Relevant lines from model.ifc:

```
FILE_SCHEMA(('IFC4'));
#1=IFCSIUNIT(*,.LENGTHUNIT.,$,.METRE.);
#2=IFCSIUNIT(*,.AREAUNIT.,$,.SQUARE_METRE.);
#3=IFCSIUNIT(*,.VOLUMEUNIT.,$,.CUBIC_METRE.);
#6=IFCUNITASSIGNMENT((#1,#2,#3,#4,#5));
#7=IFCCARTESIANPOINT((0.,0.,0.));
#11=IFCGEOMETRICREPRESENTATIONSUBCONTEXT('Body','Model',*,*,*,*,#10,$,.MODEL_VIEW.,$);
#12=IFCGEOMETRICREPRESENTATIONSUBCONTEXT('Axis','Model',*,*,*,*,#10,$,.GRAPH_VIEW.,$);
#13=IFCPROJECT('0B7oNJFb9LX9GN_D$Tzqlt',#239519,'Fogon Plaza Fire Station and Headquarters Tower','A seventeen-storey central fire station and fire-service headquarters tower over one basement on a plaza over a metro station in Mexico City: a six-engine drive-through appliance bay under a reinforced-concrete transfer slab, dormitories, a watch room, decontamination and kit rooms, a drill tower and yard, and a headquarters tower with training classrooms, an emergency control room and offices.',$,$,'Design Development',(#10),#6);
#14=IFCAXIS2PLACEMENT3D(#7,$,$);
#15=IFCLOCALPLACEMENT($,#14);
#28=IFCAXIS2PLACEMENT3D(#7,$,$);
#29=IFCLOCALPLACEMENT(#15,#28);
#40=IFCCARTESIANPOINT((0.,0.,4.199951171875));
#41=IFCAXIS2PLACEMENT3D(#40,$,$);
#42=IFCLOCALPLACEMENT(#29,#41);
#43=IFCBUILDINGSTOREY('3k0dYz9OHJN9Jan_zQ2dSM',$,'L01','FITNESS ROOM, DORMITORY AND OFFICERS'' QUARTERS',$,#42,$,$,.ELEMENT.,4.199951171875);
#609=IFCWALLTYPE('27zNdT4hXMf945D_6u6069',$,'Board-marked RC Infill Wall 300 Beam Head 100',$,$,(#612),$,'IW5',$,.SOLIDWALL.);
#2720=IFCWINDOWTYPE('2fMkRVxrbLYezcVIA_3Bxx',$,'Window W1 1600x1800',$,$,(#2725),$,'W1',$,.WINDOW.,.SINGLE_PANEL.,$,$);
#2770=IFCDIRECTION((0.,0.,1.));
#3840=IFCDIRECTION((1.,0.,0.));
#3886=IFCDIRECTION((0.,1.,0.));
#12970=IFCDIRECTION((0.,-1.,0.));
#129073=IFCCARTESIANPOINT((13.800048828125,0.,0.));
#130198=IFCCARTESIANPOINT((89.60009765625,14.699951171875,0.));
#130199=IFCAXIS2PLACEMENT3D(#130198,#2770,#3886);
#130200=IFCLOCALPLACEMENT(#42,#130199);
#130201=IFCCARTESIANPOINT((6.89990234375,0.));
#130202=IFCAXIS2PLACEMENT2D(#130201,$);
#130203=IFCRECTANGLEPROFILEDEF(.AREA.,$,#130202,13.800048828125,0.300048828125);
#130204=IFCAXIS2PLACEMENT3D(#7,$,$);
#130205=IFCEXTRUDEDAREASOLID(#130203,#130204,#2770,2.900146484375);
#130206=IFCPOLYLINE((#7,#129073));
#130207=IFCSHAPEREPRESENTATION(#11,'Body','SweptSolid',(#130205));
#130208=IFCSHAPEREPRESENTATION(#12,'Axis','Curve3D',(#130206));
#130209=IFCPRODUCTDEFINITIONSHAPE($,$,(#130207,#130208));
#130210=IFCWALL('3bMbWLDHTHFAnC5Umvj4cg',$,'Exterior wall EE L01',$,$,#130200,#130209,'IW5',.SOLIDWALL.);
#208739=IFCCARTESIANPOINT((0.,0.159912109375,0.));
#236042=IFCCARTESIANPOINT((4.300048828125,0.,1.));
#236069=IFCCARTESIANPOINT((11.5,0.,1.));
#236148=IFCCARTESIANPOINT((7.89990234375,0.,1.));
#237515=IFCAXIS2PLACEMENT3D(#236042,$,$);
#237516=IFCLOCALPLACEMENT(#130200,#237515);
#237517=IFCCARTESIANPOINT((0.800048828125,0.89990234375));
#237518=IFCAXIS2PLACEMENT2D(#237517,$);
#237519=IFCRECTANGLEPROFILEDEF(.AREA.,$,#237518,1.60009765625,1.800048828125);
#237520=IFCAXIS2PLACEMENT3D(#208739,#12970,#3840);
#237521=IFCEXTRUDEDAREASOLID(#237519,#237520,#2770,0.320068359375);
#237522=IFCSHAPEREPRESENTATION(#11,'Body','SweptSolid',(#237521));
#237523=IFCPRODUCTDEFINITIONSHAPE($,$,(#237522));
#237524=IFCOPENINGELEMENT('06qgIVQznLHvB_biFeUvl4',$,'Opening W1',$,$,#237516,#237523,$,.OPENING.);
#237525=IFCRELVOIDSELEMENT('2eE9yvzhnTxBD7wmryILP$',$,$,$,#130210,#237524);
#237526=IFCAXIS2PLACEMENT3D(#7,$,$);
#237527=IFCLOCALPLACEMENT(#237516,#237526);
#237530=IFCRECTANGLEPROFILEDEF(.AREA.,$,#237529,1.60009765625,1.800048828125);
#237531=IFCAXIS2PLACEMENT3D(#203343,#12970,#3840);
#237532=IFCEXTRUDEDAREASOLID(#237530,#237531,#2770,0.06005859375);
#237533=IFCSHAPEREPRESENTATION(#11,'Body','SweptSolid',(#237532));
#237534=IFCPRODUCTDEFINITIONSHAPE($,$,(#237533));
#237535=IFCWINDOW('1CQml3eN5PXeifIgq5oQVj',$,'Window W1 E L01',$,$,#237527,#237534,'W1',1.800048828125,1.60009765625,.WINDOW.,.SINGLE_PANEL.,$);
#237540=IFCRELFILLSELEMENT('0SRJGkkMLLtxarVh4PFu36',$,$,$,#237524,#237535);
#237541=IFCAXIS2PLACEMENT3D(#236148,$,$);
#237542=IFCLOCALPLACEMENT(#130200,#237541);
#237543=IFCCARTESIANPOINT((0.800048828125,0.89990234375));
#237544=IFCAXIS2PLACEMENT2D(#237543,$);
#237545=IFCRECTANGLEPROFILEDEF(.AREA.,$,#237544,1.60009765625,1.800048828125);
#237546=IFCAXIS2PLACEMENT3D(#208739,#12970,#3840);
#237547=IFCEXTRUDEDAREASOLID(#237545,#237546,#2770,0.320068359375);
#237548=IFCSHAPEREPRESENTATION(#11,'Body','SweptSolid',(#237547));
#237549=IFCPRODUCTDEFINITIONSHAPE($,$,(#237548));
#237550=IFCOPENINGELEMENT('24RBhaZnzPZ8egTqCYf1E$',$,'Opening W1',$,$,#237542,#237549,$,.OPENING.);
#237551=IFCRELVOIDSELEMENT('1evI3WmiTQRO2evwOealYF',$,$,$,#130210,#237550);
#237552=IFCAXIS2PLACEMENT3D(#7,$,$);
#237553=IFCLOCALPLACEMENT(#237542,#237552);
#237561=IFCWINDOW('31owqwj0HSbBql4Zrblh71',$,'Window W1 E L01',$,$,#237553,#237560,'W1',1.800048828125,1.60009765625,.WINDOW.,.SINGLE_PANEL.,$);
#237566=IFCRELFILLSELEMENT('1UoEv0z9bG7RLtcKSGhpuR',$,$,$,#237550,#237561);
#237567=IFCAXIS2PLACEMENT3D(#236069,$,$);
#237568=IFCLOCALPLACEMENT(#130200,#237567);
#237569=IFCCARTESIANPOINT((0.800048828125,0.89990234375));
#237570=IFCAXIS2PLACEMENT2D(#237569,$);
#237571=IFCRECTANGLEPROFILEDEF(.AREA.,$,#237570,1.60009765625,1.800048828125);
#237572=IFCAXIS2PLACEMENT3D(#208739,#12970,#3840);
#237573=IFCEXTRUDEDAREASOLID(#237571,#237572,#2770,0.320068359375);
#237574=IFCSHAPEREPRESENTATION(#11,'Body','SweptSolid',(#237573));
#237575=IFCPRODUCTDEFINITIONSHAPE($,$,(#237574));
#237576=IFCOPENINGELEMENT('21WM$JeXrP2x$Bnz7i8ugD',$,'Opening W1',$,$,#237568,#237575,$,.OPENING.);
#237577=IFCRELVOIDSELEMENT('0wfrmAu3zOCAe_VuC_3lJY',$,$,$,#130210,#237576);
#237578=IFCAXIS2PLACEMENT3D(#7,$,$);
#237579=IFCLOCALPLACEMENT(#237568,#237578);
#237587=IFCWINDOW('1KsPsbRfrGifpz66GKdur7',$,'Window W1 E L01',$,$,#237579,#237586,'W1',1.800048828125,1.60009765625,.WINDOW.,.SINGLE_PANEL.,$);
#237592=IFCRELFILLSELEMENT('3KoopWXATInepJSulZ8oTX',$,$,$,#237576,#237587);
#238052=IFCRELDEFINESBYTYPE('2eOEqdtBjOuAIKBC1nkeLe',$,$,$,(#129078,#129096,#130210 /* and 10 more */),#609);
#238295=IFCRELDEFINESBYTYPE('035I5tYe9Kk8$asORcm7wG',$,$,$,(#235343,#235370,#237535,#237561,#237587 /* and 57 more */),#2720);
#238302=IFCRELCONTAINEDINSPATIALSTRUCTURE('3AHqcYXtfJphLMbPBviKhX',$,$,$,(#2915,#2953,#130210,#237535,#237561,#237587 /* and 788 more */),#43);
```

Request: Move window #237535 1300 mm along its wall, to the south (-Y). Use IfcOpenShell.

```python
import ifcopenshell
import ifcopenshell.api.geometry
import ifcopenshell.util.placement
import ifcopenshell.util.unit

model = ifcopenshell.open("model.ifc")
unit_scale = ifcopenshell.util.unit.calculate_unit_scale(model)

window = model.by_guid("1CQml3eN5PXeifIgq5oQVj")
opening = window.FillsVoids[0].RelatingOpeningElement
wall = opening.VoidsElements[0].RelatingBuildingElement

wall_matrix = ifcopenshell.util.placement.get_local_placement(wall.ObjectPlacement)
shift = wall_matrix[:3, 0] * -1.3 / unit_scale
before = ifcopenshell.util.placement.get_local_placement(window.ObjectPlacement)[:3, 3].copy()

# The window is placed relative to its opening, so it follows when the opening moves.
matrix = ifcopenshell.util.placement.get_local_placement(opening.ObjectPlacement)
matrix[:3, 3] += shift
ifcopenshell.api.geometry.edit_object_placement(
    model, product=opening, matrix=matrix, is_si=False, should_transform_children=True
)

after = ifcopenshell.util.placement.get_local_placement(window.ObjectPlacement)[:3, 3]
print("window moved by", (after - before).round(3) + 0.0)

model.write("model_rev.ifc")
```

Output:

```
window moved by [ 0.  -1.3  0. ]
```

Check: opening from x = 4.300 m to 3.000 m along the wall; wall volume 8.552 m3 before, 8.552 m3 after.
